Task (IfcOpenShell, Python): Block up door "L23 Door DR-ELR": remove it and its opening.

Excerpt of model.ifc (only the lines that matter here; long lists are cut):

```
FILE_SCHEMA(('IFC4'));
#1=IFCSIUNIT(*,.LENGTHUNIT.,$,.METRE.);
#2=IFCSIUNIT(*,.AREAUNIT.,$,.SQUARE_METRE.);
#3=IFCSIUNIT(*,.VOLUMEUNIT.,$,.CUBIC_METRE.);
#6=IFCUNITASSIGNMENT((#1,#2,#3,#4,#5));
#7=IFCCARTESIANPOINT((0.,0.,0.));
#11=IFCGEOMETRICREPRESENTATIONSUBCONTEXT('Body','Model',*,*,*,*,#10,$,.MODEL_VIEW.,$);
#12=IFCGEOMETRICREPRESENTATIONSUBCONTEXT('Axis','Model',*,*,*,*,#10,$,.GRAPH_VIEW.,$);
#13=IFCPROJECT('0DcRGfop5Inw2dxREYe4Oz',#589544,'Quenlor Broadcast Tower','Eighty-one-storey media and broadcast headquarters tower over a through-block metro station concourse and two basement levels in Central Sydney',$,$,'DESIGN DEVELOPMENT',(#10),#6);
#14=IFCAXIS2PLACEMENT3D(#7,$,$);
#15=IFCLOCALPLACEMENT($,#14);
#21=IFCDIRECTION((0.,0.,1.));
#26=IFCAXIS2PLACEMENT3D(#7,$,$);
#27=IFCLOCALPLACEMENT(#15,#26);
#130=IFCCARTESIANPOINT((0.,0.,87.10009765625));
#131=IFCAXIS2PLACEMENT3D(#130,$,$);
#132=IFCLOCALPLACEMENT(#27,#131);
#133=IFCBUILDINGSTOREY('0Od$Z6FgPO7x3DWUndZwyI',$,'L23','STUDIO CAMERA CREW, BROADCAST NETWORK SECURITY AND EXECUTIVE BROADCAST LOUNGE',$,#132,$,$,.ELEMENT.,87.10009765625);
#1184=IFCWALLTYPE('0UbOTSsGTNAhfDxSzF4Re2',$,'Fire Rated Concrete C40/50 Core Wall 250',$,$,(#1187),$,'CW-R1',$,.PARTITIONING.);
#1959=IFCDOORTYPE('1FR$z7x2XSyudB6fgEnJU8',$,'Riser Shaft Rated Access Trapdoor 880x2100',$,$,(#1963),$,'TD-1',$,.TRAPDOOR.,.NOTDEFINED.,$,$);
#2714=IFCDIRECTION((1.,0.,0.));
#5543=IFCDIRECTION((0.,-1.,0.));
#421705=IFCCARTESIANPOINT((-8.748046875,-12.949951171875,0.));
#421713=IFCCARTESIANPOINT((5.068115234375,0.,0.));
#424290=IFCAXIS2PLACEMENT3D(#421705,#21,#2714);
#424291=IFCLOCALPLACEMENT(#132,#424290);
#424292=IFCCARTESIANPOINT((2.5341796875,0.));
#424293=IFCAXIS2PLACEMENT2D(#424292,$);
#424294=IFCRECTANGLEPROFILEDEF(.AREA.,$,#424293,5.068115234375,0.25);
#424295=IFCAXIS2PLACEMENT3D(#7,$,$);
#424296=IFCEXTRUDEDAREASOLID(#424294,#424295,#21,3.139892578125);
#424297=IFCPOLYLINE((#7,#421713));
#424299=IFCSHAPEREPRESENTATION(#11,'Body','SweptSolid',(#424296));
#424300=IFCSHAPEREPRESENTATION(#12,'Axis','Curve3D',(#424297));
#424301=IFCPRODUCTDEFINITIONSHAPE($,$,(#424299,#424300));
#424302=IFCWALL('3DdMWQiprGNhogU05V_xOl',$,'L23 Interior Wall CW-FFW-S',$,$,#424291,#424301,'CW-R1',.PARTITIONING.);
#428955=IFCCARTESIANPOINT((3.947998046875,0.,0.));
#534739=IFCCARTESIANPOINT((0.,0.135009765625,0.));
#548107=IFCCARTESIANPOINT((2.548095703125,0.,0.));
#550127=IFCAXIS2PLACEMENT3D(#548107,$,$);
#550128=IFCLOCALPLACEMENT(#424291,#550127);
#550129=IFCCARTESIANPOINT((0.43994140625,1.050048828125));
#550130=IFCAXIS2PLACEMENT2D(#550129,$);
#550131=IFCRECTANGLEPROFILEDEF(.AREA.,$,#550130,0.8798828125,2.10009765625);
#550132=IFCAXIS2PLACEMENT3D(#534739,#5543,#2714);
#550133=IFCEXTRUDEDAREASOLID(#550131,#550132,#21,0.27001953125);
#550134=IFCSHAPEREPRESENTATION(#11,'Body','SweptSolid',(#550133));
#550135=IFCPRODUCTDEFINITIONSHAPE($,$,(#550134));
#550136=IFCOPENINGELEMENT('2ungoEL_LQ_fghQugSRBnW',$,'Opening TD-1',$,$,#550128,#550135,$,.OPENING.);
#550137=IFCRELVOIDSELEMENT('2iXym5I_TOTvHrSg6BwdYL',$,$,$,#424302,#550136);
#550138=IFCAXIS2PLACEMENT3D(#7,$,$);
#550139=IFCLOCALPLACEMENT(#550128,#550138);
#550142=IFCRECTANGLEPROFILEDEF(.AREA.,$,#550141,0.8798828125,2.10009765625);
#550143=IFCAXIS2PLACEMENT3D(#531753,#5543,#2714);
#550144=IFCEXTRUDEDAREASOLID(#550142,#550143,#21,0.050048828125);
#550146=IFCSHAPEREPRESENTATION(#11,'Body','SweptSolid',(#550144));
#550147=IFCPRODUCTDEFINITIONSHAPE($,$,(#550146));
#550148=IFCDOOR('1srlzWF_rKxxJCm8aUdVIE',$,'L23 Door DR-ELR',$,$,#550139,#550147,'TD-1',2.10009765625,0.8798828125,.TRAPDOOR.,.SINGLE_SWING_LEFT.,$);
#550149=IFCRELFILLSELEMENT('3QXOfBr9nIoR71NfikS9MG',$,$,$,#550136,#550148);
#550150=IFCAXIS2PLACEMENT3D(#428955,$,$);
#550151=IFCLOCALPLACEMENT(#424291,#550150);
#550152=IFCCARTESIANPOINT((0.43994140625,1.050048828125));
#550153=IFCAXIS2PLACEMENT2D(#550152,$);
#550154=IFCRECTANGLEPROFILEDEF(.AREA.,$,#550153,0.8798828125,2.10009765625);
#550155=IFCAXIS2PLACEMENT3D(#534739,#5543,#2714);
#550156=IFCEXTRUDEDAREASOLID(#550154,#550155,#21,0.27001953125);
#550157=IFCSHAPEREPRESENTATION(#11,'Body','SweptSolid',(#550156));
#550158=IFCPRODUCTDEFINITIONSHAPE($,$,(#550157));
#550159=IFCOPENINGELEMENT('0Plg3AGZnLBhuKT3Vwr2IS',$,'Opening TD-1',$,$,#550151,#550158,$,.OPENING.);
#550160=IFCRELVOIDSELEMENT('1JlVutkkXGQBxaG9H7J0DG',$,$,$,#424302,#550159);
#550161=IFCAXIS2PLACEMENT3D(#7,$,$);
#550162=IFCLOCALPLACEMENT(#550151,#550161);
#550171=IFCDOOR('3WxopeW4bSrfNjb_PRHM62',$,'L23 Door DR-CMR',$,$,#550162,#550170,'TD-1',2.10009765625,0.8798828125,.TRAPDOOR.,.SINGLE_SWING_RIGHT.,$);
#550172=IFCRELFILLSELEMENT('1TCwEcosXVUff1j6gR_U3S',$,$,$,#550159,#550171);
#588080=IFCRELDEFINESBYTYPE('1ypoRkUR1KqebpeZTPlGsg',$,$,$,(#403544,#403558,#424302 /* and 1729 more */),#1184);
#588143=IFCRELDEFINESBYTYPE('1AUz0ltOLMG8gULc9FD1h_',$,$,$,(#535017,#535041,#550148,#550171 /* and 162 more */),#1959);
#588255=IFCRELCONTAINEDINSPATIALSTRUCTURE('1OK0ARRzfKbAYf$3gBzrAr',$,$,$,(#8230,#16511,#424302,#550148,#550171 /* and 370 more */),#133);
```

```python
import ifcopenshell
import ifcopenshell.api.feature
import ifcopenshell.api.root
import ifcopenshell.geom
import ifcopenshell.util.shape

model = ifcopenshell.open("model.ifc")
settings = ifcopenshell.geom.settings()


def volume(element):
    """Net volume in cubic metres, openings subtracted."""
    shape = ifcopenshell.geom.create_shape(settings, element)
    return ifcopenshell.util.shape.get_volume(shape.geometry)


door = model.by_id(550148)
opening = door.FillsVoids[0].RelatingOpeningElement
wall = opening.VoidsElements[0].RelatingBuildingElement
before = volume(wall)

ifcopenshell.api.root.remove_product(model, product=door)
ifcopenshell.api.feature.remove_feature(model, feature=opening)

after = volume(wall)

print(f"wall volume {before:.3f} -> {after:.3f} m3")

model.write("model_v2.ifc")
```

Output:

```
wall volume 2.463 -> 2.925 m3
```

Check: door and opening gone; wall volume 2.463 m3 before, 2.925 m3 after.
